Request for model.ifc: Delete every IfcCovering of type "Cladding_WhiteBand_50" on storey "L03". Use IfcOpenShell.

First a look at what the model holds.

```python
import ifcopenshell
import ifcopenshell.util.element

model = ifcopenshell.open("model.ifc")
print(model.schema)
storey = next(s for s in model.by_type("IfcBuildingStorey") if s.Name == "L03")
coverings = [e for e in ifcopenshell.util.element.get_decomposition(storey) if e.is_a("IfcCovering")]
seen = {}
for e in coverings:
    element_type = ifcopenshell.util.element.get_type(e)
    name = element_type.Name if element_type not in (None, e) else None
    seen[name] = seen.get(name, 0) + 1
for name, count in sorted(seen.items(), key=str):
    print(count, "x", name)
```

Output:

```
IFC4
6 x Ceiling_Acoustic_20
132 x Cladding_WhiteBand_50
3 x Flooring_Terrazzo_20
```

```python
import ifcopenshell
import ifcopenshell.api.root
import ifcopenshell.util.element

model = ifcopenshell.open("model.ifc")

storey = next(s for s in model.by_type("IfcBuildingStorey") if s.Name == "L03")
coverings = [e for e in ifcopenshell.util.element.get_decomposition(storey) if e.is_a("IfcCovering")]
targets = [e for e in coverings if (t := ifcopenshell.util.element.get_type(e)) not in (None, e) and t.Name == "Cladding_WhiteBand_50"]

for e in targets:
    ifcopenshell.api.root.remove_product(model, product=e)
print(len(targets), "removed")

model.write("model_v2.ifc")
```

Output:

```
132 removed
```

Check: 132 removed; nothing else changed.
